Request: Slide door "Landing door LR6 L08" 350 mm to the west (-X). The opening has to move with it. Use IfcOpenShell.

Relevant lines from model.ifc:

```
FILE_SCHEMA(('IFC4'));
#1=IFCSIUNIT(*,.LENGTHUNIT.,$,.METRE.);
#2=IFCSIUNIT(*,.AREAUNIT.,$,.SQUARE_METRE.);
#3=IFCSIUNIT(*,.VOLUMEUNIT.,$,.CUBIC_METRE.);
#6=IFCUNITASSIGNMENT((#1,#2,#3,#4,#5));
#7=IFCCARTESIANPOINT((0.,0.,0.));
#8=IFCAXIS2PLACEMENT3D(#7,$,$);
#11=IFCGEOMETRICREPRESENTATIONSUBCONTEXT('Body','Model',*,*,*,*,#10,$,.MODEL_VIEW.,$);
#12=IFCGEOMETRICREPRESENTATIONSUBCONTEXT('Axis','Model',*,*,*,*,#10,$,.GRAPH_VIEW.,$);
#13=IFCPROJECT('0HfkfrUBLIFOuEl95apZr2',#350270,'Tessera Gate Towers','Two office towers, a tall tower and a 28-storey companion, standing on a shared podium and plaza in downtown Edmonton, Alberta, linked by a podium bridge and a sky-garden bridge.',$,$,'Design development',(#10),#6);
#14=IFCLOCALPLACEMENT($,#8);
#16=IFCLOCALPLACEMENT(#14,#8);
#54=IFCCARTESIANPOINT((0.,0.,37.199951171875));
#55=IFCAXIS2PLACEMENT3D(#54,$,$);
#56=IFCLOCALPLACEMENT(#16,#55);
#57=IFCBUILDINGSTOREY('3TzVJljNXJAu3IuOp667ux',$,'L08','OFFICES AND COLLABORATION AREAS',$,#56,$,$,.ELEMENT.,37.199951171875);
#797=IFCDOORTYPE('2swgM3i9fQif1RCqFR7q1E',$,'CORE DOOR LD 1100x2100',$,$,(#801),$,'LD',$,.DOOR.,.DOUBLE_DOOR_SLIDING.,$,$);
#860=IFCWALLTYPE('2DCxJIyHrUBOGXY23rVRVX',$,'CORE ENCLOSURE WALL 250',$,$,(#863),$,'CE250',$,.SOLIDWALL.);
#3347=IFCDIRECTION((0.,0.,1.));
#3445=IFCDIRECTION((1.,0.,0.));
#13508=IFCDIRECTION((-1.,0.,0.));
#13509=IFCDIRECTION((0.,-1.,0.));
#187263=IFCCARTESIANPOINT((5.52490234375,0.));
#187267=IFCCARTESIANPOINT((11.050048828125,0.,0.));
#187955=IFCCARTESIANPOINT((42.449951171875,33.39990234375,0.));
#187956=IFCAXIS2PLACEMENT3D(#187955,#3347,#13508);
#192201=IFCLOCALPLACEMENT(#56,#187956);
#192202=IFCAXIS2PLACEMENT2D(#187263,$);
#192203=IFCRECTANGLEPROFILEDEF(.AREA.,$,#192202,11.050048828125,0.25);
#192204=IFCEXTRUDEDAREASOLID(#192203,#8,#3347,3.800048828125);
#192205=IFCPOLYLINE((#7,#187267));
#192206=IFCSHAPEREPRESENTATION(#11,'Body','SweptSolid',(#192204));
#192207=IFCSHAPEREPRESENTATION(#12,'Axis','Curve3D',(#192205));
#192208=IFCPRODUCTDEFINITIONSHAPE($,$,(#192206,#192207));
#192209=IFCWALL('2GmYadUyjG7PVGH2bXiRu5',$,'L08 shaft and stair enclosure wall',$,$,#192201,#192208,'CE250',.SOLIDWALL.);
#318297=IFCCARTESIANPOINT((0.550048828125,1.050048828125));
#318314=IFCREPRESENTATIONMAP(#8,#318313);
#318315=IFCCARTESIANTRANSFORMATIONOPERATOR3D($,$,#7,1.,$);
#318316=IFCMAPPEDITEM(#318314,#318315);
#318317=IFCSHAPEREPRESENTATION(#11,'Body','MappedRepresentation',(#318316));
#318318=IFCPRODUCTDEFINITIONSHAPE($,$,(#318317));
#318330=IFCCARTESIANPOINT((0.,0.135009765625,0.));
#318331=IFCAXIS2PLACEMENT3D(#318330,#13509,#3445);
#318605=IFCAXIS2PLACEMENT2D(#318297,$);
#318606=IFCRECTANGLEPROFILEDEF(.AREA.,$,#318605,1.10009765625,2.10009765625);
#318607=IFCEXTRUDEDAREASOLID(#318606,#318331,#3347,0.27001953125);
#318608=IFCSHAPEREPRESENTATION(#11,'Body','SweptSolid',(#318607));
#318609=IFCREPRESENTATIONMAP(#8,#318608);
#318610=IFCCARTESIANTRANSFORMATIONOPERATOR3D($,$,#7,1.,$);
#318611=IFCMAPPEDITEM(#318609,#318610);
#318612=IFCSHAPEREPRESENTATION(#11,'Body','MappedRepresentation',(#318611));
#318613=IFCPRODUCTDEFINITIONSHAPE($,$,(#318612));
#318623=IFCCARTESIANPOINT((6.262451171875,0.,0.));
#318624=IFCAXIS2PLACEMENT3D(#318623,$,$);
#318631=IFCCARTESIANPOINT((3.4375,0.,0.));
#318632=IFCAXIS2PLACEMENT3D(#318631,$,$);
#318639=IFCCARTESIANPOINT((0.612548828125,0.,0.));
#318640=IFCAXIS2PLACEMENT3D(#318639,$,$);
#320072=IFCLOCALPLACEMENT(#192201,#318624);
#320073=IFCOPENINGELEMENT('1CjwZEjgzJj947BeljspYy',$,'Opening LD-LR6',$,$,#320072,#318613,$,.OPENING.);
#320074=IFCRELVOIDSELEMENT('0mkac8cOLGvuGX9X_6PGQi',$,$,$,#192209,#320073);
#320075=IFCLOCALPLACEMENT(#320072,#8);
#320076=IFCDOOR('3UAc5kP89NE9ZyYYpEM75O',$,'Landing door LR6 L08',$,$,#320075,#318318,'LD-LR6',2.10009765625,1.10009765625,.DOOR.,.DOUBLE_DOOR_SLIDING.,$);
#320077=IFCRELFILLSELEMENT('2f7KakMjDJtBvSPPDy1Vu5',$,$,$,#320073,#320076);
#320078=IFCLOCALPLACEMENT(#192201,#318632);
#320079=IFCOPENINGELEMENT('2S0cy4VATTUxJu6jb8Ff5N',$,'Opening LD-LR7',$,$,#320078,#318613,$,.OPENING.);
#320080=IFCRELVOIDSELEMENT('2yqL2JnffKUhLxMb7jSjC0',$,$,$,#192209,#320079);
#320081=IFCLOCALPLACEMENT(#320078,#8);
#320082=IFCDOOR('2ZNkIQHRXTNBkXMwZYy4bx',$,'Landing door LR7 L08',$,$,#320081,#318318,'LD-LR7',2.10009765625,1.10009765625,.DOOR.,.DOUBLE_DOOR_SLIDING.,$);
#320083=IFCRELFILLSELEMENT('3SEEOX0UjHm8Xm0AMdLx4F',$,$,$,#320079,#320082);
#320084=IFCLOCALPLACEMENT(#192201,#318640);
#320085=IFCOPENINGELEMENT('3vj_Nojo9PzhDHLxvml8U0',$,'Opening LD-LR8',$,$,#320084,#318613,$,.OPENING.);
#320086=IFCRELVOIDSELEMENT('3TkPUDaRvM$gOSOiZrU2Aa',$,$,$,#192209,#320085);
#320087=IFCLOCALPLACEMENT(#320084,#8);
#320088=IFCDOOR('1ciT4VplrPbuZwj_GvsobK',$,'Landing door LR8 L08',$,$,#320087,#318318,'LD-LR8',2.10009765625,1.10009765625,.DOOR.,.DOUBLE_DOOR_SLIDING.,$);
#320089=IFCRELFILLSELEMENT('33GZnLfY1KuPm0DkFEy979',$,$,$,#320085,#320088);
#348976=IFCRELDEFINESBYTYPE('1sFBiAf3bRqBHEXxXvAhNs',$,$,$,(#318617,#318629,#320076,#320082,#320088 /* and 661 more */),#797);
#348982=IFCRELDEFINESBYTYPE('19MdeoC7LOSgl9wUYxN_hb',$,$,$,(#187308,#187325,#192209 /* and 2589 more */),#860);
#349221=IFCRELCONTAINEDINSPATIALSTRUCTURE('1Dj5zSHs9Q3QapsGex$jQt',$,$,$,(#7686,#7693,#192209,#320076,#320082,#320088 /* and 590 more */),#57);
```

```python
import ifcopenshell
import ifcopenshell.api.geometry
import ifcopenshell.util.placement
import ifcopenshell.util.unit

model = ifcopenshell.open("model.ifc")
unit_scale = ifcopenshell.util.unit.calculate_unit_scale(model)

door = model.by_id(320076)
opening = door.FillsVoids[0].RelatingOpeningElement
wall = opening.VoidsElements[0].RelatingBuildingElement

wall_matrix = ifcopenshell.util.placement.get_local_placement(wall.ObjectPlacement)
shift = wall_matrix[:3, 0] * 0.35 / unit_scale
before = ifcopenshell.util.placement.get_local_placement(door.ObjectPlacement)[:3, 3].copy()

# The door is placed relative to its opening, so it follows when the opening moves.
matrix = ifcopenshell.util.placement.get_local_placement(opening.ObjectPlacement)
matrix[:3, 3] += shift
ifcopenshell.api.geometry.edit_object_placement(
    model, product=opening, matrix=matrix, is_si=False, should_transform_children=True
)

after = ifcopenshell.util.placement.get_local_placement(door.ObjectPlacement)[:3, 3]
print("door moved by", (after - before).round(3) + 0.0)

model.write("model_updated.ifc")
```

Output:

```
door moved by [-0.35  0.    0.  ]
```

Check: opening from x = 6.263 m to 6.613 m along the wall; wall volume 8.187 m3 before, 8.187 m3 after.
